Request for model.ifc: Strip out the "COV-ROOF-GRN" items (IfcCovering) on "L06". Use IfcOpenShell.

First a look at what the model holds.

```python
import ifcopenshell
import ifcopenshell.util.element

model = ifcopenshell.open("model.ifc")
print(model.schema)
storey = next(s for s in model.by_type("IfcBuildingStorey") if s.Name == "L06")
coverings = [e for e in ifcopenshell.util.element.get_decomposition(storey) if e.is_a("IfcCovering")]
seen = {}
for e in coverings:
    element_type = ifcopenshell.util.element.get_type(e)
    name = element_type.Name if element_type not in (None, e) else None
    seen[name] = seen.get(name, 0) + 1
for name, count in sorted(seen.items(), key=str):
    print(count, "x", name)
```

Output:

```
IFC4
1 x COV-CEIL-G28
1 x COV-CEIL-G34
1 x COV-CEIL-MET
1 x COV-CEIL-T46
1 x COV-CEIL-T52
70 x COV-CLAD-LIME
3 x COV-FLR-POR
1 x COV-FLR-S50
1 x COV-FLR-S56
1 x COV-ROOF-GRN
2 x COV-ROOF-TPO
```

```python
import ifcopenshell
import ifcopenshell.api.root
import ifcopenshell.util.element

model = ifcopenshell.open("model.ifc")

storey = next(s for s in model.by_type("IfcBuildingStorey") if s.Name == "L06")
coverings = [e for e in ifcopenshell.util.element.get_decomposition(storey) if e.is_a("IfcCovering")]
targets = [e for e in coverings if (t := ifcopenshell.util.element.get_type(e)) not in (None, e) and t.Name == "COV-ROOF-GRN"]

for e in targets:
    ifcopenshell.api.root.remove_product(model, product=e)
print(len(targets), "removed")

model.write("model_rev.ifc")
```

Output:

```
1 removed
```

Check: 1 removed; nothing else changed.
